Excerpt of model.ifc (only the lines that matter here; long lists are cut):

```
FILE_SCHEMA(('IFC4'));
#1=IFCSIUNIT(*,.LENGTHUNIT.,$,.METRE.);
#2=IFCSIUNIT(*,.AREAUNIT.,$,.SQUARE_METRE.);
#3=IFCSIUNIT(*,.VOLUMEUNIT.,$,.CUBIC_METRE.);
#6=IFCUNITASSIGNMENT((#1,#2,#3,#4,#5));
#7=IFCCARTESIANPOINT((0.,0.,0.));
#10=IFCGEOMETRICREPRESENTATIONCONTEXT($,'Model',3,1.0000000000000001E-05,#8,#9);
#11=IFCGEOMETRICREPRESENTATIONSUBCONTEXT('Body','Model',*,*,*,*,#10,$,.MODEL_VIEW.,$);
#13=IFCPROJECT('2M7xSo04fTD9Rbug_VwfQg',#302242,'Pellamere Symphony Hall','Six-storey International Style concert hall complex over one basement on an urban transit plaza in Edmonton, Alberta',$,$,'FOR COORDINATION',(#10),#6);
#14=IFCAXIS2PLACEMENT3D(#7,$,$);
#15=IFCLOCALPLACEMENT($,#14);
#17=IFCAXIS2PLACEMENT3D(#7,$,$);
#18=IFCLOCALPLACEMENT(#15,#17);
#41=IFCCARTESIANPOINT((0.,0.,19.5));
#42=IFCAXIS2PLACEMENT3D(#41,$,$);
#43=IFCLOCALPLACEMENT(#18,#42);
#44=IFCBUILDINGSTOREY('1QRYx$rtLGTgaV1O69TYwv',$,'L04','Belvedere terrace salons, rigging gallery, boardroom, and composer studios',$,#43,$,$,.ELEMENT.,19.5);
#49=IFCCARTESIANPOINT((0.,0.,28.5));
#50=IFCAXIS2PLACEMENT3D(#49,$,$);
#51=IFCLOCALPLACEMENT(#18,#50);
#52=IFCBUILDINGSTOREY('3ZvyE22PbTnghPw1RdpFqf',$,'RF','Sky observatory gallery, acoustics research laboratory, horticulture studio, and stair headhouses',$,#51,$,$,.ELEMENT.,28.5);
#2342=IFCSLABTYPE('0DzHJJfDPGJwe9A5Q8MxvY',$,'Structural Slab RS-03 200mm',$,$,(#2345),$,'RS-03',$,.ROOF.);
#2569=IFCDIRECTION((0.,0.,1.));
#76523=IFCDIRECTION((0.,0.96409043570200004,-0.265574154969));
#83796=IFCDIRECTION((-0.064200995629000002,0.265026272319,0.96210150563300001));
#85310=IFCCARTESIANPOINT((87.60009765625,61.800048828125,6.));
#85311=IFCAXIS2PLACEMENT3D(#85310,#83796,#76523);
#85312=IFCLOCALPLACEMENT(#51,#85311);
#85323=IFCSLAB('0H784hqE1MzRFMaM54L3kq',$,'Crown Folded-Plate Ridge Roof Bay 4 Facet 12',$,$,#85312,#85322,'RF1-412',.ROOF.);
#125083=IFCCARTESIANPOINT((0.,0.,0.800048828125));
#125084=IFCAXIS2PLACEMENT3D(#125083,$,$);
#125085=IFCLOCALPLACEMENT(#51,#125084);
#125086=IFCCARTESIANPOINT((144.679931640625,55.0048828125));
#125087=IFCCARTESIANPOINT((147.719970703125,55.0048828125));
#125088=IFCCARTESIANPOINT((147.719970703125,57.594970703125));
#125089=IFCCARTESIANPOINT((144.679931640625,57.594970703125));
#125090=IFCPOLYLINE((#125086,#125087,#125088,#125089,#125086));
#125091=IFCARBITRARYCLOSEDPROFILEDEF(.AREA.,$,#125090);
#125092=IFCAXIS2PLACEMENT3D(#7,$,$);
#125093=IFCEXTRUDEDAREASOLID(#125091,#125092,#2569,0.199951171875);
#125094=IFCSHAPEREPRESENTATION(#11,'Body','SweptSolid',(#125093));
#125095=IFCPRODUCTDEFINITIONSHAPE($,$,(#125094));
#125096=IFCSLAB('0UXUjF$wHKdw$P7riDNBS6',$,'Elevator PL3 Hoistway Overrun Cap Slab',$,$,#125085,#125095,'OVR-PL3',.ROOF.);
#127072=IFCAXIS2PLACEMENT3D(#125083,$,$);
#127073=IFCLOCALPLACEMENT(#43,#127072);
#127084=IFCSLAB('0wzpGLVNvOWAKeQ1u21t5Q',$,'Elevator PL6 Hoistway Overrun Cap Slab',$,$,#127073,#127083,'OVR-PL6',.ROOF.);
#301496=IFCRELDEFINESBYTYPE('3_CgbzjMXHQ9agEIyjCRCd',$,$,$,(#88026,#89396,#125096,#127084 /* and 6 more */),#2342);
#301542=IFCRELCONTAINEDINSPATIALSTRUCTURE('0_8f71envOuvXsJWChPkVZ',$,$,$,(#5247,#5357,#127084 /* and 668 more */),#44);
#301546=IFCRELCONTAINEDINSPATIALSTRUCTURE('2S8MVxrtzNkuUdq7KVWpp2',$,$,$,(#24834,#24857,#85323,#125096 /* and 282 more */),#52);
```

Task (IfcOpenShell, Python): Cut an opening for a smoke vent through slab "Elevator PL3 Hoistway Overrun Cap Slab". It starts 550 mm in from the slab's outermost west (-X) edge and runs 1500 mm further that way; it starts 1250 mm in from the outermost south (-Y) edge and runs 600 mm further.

```python
import numpy as np
import ifcopenshell
import ifcopenshell.api.feature
import ifcopenshell.api.geometry
import ifcopenshell.api.root
import ifcopenshell.geom
import ifcopenshell.util.placement
import ifcopenshell.util.representation
import ifcopenshell.util.shape
import ifcopenshell.util.unit

model = ifcopenshell.open("model.ifc")
unit_scale = ifcopenshell.util.unit.calculate_unit_scale(model)
settings = ifcopenshell.geom.settings()


def volume(element):
    """Net volume in cubic metres, openings subtracted."""
    shape = ifcopenshell.geom.create_shape(settings, element)
    return ifcopenshell.util.shape.get_volume(shape.geometry)


slab = model.by_guid("0UXUjF$wHKdw$P7riDNBS6")
before = volume(slab)

# Extent in the slab's own axes, in metres. The edges named are its -X and -Y sides.
slab_shape = ifcopenshell.geom.create_shape(settings, slab)
vertices = ifcopenshell.util.shape.get_vertices(slab_shape.geometry)
x_min, y_min, bottom = vertices.min(axis=0)
top = vertices[:, 2].max()

opening = ifcopenshell.api.root.create_entity(model, ifc_class="IfcOpeningElement", name="Smoke vent opening", predefined_type="OPENING")
context = ifcopenshell.util.representation.get_context(model, "Model", "Body", "MODEL_VIEW")
width, depth = 1.5, 0.6
outline = [(0.0, 0.0), (width, 0.0), (width, depth), (0.0, depth), (0.0, 0.0)]
# Overshoot both faces by 50 mm so the cut is clean.
shape = ifcopenshell.api.geometry.add_slab_representation(
    model, context=context, depth=top - bottom + 0.1, polyline=outline
)
ifcopenshell.api.geometry.assign_representation(model, product=opening, representation=shape)

matrix = ifcopenshell.util.placement.get_local_placement(slab.ObjectPlacement)
matrix[:, 3] = matrix @ np.append(np.array([x_min + 0.55, y_min + 1.25, bottom - 0.05]) / unit_scale, 1.0)
ifcopenshell.api.geometry.edit_object_placement(model, product=opening, matrix=matrix, is_si=False)
ifcopenshell.api.feature.add_feature(model, feature=opening, element=slab)

after = volume(slab)

print(f"slab volume {before:.3f} -> {after:.3f} m3")

model.write("model_v2.ifc")
```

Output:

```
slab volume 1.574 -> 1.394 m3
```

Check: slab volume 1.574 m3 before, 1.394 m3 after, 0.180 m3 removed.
